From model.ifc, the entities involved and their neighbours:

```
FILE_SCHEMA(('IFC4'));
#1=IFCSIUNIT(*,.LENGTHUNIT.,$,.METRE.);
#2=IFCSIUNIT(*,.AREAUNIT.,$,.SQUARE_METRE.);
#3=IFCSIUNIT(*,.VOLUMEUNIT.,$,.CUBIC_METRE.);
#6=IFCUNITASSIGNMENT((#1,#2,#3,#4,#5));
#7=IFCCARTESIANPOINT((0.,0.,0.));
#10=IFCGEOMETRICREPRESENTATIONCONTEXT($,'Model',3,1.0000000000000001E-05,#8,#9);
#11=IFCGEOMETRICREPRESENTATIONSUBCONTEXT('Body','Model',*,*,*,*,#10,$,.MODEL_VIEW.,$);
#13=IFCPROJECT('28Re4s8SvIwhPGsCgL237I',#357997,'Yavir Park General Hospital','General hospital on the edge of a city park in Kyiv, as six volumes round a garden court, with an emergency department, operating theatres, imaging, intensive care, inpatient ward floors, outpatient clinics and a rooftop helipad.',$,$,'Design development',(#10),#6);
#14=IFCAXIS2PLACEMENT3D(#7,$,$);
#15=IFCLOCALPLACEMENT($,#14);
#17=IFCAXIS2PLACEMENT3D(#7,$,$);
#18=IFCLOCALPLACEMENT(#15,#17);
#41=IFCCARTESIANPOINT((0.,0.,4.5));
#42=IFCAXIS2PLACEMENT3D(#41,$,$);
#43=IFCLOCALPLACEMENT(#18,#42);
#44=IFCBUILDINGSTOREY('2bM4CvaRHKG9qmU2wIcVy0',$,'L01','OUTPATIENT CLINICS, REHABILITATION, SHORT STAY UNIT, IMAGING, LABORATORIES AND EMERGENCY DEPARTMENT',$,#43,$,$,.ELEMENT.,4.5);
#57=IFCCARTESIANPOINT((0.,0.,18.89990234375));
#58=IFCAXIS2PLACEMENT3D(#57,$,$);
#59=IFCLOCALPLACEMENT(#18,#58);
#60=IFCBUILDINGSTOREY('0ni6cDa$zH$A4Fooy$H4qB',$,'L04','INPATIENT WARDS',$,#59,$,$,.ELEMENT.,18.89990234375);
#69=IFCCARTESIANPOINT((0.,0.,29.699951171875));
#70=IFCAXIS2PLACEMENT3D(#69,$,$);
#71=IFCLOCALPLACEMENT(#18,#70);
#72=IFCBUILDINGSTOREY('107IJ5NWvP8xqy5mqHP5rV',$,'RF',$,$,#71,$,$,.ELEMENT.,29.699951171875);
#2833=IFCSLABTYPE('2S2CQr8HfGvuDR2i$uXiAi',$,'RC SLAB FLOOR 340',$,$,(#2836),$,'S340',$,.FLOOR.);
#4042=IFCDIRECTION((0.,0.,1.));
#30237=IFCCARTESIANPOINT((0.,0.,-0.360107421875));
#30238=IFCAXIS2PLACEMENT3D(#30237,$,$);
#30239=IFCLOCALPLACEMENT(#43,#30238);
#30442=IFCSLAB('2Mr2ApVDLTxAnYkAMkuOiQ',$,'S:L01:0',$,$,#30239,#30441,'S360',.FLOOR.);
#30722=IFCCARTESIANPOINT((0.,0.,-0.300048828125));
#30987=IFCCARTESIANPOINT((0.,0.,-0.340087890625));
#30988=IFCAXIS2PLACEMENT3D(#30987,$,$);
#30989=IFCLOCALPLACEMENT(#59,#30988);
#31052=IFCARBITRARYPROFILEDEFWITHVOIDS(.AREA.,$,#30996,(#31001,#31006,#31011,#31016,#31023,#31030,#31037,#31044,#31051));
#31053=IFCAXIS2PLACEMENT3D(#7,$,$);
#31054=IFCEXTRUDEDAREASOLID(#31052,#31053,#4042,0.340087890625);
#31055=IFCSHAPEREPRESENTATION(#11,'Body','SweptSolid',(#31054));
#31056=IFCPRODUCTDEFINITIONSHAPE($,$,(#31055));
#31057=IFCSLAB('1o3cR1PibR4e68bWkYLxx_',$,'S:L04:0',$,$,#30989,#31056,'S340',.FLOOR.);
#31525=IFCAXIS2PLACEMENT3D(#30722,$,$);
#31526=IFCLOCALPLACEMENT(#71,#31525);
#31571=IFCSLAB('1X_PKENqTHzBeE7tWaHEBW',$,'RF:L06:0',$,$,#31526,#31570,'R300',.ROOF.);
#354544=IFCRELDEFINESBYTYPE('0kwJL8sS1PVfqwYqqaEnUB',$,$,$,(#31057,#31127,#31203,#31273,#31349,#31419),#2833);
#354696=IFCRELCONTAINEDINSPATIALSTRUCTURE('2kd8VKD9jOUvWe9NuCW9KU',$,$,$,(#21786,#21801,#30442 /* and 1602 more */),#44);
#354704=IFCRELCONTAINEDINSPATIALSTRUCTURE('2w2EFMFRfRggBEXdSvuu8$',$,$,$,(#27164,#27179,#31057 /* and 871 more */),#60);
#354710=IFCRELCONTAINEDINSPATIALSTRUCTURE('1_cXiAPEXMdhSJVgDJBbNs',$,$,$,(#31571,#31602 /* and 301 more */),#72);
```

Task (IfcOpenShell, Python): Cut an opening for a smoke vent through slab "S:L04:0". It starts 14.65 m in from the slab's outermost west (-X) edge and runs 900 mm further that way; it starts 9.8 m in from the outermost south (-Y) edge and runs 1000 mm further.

```python
import numpy as np
import ifcopenshell
import ifcopenshell.api.feature
import ifcopenshell.api.geometry
import ifcopenshell.api.root
import ifcopenshell.geom
import ifcopenshell.util.placement
import ifcopenshell.util.representation
import ifcopenshell.util.shape
import ifcopenshell.util.unit

model = ifcopenshell.open("model.ifc")
unit_scale = ifcopenshell.util.unit.calculate_unit_scale(model)
settings = ifcopenshell.geom.settings()


def volume(element):
    """Net volume in cubic metres, openings subtracted."""
    shape = ifcopenshell.geom.create_shape(settings, element)
    return ifcopenshell.util.shape.get_volume(shape.geometry)


slab = model.by_guid("1o3cR1PibR4e68bWkYLxx_")
before = volume(slab)

# Extent in the slab's own axes, in metres. The edges named are its -X and -Y sides.
slab_shape = ifcopenshell.geom.create_shape(settings, slab)
vertices = ifcopenshell.util.shape.get_vertices(slab_shape.geometry)
x_min, y_min, bottom = vertices.min(axis=0)
top = vertices[:, 2].max()

opening = ifcopenshell.api.root.create_entity(model, ifc_class="IfcOpeningElement", name="Smoke vent opening", predefined_type="OPENING")
context = ifcopenshell.util.representation.get_context(model, "Model", "Body", "MODEL_VIEW")
width, depth = 0.9, 1
outline = [(0.0, 0.0), (width, 0.0), (width, depth), (0.0, depth), (0.0, 0.0)]
# Overshoot both faces by 50 mm so the cut is clean.
shape = ifcopenshell.api.geometry.add_slab_representation(
    model, context=context, depth=top - bottom + 0.1, polyline=outline
)
ifcopenshell.api.geometry.assign_representation(model, product=opening, representation=shape)

matrix = ifcopenshell.util.placement.get_local_placement(slab.ObjectPlacement)
matrix[:, 3] = matrix @ np.append(np.array([x_min + 14.65, y_min + 9.8, bottom - 0.05]) / unit_scale, 1.0)
ifcopenshell.api.geometry.edit_object_placement(model, product=opening, matrix=matrix, is_si=False)
ifcopenshell.api.feature.add_feature(model, feature=opening, element=slab)

after = volume(slab)

print(f"slab volume {before:.3f} -> {after:.3f} m3")

model.write("model_v2.ifc")
```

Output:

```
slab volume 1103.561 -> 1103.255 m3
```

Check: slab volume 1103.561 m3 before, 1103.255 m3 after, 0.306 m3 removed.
